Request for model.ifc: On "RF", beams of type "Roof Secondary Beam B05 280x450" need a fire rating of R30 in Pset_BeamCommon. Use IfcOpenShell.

First a look at what the model holds.

```python
import ifcopenshell
import ifcopenshell.util.element

model = ifcopenshell.open("model.ifc")
print(model.schema)
storey = next(s for s in model.by_type("IfcBuildingStorey") if s.Name == "RF")
beams = [e for e in ifcopenshell.util.element.get_decomposition(storey) if e.is_a("IfcBeam")]
seen = {}
for e in beams:
    element_type = ifcopenshell.util.element.get_type(e)
    key = (element_type.Name if element_type != e and element_type else None, ifcopenshell.util.element.get_pset(e, "Pset_BeamCommon", "FireRating"))
    seen[key] = seen.get(key, 0) + 1
for (name, value), count in sorted(seen.items(), key=str):
    print(count, "x", name, "|", value)
```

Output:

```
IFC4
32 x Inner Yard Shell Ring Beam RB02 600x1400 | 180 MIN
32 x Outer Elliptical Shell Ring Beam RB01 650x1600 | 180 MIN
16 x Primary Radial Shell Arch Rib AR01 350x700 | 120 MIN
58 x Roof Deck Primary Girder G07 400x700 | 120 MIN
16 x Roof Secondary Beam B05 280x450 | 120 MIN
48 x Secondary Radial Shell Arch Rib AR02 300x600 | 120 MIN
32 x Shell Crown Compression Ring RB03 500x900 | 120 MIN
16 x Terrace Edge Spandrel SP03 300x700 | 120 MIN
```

```python
import ifcopenshell
import ifcopenshell.api.pset
import ifcopenshell.util.element

model = ifcopenshell.open("model.ifc")

storey = next(s for s in model.by_type("IfcBuildingStorey") if s.Name == "RF")
beams = [e for e in ifcopenshell.util.element.get_decomposition(storey) if e.is_a("IfcBeam")]

count = 0
for e in beams:
    element_type = ifcopenshell.util.element.get_type(e)
    if element_type in (None, e) or element_type.Name != "Roof Secondary Beam B05 280x450":
        continue
    # add_pset returns the element's existing set when there is one.
    pset = ifcopenshell.api.pset.add_pset(model, product=e, name="Pset_BeamCommon")
    ifcopenshell.api.pset.edit_pset(model, pset=pset, properties={"FireRating": "R30"})
    count += 1

print(count, "beams updated")

model.write("model_edited.ifc")
```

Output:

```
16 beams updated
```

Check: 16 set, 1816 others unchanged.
